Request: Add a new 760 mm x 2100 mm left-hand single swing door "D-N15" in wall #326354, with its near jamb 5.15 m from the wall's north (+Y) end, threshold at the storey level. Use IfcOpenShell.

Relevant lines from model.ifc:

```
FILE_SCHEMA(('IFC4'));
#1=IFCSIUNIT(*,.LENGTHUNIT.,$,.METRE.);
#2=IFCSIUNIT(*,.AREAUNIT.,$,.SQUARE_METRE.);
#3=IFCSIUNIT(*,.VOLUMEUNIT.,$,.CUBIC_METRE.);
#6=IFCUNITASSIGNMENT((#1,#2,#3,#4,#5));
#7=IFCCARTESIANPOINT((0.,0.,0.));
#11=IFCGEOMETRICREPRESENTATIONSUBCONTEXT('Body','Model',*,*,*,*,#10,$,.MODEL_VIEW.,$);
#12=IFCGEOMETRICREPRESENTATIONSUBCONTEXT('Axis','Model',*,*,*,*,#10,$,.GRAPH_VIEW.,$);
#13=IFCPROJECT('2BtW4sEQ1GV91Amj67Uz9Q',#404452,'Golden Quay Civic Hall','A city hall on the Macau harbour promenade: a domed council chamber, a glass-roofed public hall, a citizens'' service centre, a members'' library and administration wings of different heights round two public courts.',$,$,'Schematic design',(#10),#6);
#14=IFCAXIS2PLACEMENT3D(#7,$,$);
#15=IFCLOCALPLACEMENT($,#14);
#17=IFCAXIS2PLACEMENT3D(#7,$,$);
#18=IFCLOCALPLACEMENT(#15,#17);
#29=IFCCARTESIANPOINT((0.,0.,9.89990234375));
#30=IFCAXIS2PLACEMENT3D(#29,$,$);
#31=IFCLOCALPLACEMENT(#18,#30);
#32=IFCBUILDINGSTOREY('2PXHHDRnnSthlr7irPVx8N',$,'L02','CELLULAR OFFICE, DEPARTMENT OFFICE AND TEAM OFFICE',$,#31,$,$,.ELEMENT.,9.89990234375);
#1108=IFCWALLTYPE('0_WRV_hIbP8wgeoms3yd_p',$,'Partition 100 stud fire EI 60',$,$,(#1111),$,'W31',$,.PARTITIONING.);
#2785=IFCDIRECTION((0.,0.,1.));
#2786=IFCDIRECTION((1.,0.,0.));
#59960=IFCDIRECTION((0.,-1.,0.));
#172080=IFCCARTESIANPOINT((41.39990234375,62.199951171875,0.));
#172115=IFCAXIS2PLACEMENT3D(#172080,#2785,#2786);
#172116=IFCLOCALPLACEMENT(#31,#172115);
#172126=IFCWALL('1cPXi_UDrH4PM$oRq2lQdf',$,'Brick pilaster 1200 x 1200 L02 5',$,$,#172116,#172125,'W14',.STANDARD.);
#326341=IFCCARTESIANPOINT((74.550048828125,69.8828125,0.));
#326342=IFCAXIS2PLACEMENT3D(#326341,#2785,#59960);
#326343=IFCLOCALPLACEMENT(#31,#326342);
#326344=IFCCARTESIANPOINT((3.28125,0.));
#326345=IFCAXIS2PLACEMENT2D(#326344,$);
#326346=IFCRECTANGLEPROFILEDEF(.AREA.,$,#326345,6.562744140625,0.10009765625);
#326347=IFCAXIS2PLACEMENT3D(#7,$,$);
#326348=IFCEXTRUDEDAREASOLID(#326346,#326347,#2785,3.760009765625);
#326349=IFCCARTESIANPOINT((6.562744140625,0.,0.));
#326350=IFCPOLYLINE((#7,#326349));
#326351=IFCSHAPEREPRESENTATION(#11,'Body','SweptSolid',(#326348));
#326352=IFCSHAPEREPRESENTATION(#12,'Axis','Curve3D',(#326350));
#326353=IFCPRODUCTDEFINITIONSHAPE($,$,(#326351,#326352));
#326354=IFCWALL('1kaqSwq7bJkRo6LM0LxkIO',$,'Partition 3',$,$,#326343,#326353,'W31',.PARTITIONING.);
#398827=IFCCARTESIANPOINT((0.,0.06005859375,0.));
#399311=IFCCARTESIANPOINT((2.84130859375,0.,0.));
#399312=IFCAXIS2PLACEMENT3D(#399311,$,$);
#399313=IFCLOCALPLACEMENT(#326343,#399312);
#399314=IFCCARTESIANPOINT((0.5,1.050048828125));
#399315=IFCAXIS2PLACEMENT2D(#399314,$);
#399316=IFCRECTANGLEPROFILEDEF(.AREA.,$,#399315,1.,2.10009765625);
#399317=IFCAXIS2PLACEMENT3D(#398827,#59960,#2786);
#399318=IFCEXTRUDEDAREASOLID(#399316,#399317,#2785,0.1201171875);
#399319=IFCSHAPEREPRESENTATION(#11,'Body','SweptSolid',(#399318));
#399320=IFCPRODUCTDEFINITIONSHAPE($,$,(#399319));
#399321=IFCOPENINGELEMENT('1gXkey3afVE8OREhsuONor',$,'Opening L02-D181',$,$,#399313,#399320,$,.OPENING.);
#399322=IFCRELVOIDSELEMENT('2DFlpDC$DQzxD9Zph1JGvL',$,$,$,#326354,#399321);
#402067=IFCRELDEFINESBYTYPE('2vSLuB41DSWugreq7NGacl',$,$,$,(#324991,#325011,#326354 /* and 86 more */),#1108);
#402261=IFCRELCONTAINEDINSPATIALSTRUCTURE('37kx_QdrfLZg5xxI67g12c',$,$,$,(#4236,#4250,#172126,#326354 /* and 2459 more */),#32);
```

```python
import numpy as np
import ifcopenshell
import ifcopenshell.api.feature
import ifcopenshell.api.geometry
import ifcopenshell.api.root
import ifcopenshell.api.spatial
import ifcopenshell.geom
import ifcopenshell.util.element
import ifcopenshell.util.placement
import ifcopenshell.util.representation
import ifcopenshell.util.shape
import ifcopenshell.util.unit

model = ifcopenshell.open("model.ifc")
unit_scale = ifcopenshell.util.unit.calculate_unit_scale(model)
settings = ifcopenshell.geom.settings()


def volume(element):
    """Net volume in cubic metres, openings subtracted."""
    shape = ifcopenshell.geom.create_shape(settings, element)
    return ifcopenshell.util.shape.get_volume(shape.geometry)


wall = model.by_guid("1kaqSwq7bJkRo6LM0LxkIO")
storey = ifcopenshell.util.element.get_container(wall, ifc_class="IfcBuildingStorey")
context = ifcopenshell.util.representation.get_context(model, "Model", "Body", "MODEL_VIEW")
before = volume(wall)

width, height, from_end, sill = 0.76, 2.1, 5.15, 0.0  # metres

# The wall runs along its own X axis, and the end named is its -X end.
wall_shape = ifcopenshell.geom.create_shape(settings, wall)
x, y, z = ifcopenshell.util.shape.get_vertices(wall_shape.geometry).T
start = x.min() + from_end
face, thickness = float(y.min()), float(y.max() - y.min())
wall_matrix = ifcopenshell.util.placement.get_local_placement(wall.ObjectPlacement)
level = ifcopenshell.util.placement.get_local_placement(storey.ObjectPlacement)[2, 3]


def in_wall(x, y):
    """Placement at x, y metres in the wall's axes, at sill height."""
    matrix = wall_matrix.copy()
    matrix[:, 3] = wall_matrix @ np.array([x / unit_scale, y / unit_scale, 0.0, 1.0])
    matrix[2, 3] = level + sill / unit_scale
    return matrix


# Opening: a box that overshoots both wall faces by 50 mm.
opening = ifcopenshell.api.root.create_entity(model, ifc_class="IfcOpeningElement", predefined_type="OPENING")
box = ifcopenshell.api.geometry.add_wall_representation(
    model, context=context, length=width, height=height, thickness=thickness + 0.1
)
ifcopenshell.api.geometry.assign_representation(model, product=opening, representation=box)
ifcopenshell.api.geometry.edit_object_placement(model, product=opening, matrix=in_wall(start, face - 0.05), is_si=False)
ifcopenshell.api.feature.add_feature(model, feature=opening, element=wall)

door = ifcopenshell.api.root.create_entity(model, ifc_class="IfcDoor", name="D-N15", predefined_type="DOOR")
door.OverallWidth, door.OverallHeight = width / unit_scale, height / unit_scale
door.OperationType = "SINGLE_SWING_LEFT"
body = ifcopenshell.api.geometry.add_door_representation(
    model,
    context=context,
    overall_width=door.OverallWidth,
    overall_height=door.OverallHeight,
    operation_type="SINGLE_SWING_LEFT",
    lining_properties={"LiningDepth": thickness / unit_scale, "ThresholdDepth": thickness / unit_scale},
)
ifcopenshell.api.geometry.assign_representation(model, product=door, representation=body)
ifcopenshell.api.spatial.assign_container(model, products=[door], relating_structure=storey)
ifcopenshell.api.feature.add_filling(model, opening=opening, element=door)

# The lining spans the wall, so the door starts at the wall face.
ifcopenshell.api.geometry.edit_object_placement(model, product=door, matrix=in_wall(start, face), is_si=False)

after = volume(wall)

print(f"wall volume {before:.3f} -> {after:.3f} m3")

model.write("model_updated.ifc")
```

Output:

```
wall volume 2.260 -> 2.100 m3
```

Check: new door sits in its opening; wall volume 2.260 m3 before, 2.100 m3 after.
